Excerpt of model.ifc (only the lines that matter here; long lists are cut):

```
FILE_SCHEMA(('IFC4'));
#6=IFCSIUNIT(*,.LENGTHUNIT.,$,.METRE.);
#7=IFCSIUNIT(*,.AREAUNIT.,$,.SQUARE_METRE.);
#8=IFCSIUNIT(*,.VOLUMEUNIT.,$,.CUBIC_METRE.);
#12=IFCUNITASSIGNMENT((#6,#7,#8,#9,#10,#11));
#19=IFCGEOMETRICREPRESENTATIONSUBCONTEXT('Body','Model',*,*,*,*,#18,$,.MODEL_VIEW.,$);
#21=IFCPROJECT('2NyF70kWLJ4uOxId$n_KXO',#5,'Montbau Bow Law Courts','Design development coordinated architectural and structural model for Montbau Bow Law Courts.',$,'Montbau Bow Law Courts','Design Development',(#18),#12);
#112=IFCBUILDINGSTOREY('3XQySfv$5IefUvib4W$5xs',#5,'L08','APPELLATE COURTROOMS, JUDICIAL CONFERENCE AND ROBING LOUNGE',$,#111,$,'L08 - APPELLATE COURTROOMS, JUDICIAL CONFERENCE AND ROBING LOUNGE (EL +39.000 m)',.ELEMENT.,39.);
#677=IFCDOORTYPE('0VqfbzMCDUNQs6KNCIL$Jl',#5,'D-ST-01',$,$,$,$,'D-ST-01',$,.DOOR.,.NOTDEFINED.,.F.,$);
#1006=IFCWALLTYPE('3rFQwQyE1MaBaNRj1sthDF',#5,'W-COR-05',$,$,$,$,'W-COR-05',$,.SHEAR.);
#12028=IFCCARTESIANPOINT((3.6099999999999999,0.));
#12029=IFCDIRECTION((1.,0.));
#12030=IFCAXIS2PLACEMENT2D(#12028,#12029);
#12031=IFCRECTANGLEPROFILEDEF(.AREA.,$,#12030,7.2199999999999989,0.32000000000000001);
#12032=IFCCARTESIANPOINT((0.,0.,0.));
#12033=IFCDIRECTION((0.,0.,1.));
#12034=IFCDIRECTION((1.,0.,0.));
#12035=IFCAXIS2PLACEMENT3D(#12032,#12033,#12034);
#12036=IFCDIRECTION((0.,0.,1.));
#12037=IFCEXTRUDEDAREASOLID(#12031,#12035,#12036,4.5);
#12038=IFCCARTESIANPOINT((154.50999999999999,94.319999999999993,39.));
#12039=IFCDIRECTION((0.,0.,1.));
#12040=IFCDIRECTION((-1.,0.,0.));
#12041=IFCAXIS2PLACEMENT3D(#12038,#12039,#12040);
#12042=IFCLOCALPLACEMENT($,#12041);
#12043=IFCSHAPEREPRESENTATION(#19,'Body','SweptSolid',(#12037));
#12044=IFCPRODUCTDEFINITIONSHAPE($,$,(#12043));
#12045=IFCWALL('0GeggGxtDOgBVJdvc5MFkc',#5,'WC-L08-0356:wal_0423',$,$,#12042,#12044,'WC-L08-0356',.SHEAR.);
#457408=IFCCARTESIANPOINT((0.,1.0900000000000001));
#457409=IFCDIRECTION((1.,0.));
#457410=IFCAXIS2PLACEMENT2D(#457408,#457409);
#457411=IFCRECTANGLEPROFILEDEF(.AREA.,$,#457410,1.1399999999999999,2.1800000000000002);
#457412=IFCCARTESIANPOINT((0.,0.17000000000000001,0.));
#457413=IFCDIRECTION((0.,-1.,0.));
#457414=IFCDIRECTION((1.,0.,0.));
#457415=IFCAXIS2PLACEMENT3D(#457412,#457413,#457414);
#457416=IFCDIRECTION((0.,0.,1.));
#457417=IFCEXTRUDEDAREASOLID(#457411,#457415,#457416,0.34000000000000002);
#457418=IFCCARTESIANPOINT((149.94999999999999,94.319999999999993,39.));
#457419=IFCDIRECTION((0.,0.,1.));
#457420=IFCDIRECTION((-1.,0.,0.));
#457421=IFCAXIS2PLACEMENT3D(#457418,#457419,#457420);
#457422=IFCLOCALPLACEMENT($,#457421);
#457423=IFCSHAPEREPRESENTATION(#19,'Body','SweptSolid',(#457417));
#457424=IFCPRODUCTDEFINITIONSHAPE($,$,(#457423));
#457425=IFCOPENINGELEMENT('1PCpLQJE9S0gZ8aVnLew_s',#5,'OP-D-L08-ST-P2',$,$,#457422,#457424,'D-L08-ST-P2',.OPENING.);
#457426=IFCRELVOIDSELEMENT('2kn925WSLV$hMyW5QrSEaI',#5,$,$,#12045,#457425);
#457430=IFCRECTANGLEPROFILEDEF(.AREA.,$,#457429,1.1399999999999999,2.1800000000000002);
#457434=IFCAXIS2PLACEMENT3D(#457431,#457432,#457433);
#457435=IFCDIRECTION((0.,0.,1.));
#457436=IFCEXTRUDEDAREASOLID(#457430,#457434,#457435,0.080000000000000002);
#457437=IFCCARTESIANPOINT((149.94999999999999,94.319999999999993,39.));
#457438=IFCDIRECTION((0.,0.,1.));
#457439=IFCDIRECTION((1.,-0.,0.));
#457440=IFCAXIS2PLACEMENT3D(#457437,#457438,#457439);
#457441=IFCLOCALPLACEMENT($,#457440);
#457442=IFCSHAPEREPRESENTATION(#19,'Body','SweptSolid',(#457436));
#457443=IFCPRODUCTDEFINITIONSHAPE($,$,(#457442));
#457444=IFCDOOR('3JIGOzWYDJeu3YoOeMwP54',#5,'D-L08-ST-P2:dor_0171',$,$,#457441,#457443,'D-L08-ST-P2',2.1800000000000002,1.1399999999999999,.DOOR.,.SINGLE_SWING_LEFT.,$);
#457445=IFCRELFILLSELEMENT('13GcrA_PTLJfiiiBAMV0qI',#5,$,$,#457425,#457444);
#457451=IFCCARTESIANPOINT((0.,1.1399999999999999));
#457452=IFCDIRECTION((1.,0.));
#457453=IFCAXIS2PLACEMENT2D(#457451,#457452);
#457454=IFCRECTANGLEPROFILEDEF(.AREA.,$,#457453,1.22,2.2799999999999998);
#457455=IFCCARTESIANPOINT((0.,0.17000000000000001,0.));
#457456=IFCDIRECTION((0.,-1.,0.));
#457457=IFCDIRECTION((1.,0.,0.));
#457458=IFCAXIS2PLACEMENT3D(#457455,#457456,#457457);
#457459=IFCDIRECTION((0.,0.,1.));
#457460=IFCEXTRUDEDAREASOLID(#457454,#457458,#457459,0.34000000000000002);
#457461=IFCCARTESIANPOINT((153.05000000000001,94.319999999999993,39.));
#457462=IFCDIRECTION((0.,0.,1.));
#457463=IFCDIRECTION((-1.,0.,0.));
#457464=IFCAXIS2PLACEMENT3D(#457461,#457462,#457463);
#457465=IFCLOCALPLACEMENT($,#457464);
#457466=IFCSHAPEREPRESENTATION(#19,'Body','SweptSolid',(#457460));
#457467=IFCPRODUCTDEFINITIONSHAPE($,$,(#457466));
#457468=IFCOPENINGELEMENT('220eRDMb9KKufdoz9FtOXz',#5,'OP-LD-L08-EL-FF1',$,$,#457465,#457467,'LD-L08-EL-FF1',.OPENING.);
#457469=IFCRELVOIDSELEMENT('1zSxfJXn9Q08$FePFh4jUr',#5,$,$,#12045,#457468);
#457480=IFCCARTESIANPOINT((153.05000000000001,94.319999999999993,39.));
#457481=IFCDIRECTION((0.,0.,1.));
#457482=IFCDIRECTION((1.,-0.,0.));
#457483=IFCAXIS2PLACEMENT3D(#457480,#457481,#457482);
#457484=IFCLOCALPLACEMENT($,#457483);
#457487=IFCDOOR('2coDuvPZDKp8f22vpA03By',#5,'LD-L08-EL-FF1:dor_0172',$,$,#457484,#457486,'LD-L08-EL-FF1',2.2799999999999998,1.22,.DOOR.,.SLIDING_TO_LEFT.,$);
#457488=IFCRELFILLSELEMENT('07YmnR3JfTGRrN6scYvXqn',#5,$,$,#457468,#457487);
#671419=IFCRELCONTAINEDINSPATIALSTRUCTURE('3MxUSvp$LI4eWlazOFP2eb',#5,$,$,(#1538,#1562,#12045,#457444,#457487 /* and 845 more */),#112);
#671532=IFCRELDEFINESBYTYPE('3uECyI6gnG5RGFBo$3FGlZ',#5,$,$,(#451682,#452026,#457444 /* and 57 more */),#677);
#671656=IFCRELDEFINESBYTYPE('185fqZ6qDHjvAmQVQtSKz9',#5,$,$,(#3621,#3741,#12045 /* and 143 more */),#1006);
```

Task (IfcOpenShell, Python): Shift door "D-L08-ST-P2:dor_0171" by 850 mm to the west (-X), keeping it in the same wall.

```python
import ifcopenshell
import ifcopenshell.api.geometry
import ifcopenshell.util.placement
import ifcopenshell.util.unit

model = ifcopenshell.open("model.ifc")
unit_scale = ifcopenshell.util.unit.calculate_unit_scale(model)

door = model.by_id(457444)
opening = door.FillsVoids[0].RelatingOpeningElement
wall = opening.VoidsElements[0].RelatingBuildingElement

wall_matrix = ifcopenshell.util.placement.get_local_placement(wall.ObjectPlacement)
shift = wall_matrix[:3, 0] * 0.85 / unit_scale
before = ifcopenshell.util.placement.get_local_placement(door.ObjectPlacement)[:3, 3].copy()

# The door is not placed relative to its opening, so move both.
for product in (opening, door):
    matrix = ifcopenshell.util.placement.get_local_placement(product.ObjectPlacement)
    matrix[:3, 3] += shift
    ifcopenshell.api.geometry.edit_object_placement(model, product=product, matrix=matrix, is_si=False)

after = ifcopenshell.util.placement.get_local_placement(door.ObjectPlacement)[:3, 3]
print("door moved by", (after - before).round(3) + 0.0)

model.write("model_rev.ifc")
```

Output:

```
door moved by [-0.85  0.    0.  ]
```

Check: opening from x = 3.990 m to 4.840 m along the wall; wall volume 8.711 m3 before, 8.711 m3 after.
